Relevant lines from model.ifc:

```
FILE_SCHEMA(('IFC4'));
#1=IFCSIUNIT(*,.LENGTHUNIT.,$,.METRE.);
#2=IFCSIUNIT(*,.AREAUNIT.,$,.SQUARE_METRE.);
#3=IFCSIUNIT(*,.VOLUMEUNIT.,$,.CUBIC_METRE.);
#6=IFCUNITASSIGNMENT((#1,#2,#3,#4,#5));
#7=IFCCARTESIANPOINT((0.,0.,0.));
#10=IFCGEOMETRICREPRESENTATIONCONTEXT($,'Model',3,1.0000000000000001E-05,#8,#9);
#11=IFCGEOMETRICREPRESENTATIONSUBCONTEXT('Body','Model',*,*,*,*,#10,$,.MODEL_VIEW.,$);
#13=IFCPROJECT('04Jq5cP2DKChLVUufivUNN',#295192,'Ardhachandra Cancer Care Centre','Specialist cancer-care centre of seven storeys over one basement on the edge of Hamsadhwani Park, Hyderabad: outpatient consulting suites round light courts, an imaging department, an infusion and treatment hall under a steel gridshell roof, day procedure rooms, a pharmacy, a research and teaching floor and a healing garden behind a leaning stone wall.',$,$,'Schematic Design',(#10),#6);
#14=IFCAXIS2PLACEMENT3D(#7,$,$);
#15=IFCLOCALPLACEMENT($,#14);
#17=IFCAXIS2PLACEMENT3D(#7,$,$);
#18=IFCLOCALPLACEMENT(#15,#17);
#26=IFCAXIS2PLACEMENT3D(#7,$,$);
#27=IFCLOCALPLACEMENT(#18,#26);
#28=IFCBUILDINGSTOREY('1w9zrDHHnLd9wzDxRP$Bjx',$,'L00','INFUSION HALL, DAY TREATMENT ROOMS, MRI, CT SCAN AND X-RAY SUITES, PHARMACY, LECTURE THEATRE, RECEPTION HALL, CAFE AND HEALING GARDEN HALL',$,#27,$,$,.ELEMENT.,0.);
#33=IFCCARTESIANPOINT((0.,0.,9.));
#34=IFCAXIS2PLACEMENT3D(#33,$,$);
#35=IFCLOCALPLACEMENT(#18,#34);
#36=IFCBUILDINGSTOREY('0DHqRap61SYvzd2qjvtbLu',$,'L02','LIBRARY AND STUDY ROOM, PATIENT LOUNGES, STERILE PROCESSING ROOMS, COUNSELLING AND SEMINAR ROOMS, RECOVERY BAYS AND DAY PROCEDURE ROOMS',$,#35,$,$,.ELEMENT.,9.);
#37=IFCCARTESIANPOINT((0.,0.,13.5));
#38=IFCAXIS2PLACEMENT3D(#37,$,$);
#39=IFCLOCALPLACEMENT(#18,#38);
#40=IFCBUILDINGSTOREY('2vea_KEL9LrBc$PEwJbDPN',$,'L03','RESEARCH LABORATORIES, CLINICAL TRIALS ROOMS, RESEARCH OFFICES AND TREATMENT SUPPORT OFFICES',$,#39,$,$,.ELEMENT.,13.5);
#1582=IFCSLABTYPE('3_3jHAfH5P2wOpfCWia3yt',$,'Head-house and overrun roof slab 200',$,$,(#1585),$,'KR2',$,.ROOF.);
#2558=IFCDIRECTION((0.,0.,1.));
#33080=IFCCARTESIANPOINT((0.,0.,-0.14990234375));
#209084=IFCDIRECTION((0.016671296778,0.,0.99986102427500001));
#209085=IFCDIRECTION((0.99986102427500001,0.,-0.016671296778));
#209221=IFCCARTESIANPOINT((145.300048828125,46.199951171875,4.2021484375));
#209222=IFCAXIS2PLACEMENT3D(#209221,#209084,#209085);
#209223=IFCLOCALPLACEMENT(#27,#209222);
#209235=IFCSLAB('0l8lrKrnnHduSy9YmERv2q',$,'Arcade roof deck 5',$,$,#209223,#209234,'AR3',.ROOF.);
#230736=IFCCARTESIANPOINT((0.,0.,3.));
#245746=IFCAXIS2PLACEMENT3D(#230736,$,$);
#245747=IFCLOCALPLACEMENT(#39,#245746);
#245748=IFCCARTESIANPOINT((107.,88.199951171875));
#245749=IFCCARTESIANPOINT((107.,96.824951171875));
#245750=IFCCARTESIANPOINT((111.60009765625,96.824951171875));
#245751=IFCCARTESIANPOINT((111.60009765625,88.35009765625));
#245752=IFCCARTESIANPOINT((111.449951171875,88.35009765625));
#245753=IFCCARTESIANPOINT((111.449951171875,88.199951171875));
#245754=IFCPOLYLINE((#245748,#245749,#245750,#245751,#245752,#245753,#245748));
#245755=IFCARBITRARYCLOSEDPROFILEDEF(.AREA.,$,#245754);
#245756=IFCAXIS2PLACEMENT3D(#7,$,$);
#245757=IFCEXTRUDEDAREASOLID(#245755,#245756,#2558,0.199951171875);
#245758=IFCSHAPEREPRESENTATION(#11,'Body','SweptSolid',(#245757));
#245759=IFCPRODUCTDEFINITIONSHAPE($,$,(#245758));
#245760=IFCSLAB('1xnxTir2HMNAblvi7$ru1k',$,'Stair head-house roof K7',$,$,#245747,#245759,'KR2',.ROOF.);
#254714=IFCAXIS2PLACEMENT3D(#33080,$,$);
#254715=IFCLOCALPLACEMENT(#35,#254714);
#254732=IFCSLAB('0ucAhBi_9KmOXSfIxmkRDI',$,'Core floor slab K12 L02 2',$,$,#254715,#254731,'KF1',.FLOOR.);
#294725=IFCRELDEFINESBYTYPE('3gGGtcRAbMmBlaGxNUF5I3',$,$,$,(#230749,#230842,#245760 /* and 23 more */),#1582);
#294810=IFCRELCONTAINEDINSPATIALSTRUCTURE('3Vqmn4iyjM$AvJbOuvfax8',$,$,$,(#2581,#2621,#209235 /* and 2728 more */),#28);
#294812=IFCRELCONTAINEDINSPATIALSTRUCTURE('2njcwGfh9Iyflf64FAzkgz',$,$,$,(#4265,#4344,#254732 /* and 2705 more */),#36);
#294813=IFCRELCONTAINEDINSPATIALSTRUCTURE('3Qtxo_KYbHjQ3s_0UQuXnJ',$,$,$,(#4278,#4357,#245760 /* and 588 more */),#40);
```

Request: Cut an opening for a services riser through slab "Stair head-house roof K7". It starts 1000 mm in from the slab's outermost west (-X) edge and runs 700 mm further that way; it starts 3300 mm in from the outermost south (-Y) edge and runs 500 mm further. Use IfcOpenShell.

```python
import numpy as np
import ifcopenshell
import ifcopenshell.api.feature
import ifcopenshell.api.geometry
import ifcopenshell.api.root
import ifcopenshell.geom
import ifcopenshell.util.placement
import ifcopenshell.util.representation
import ifcopenshell.util.shape
import ifcopenshell.util.unit

model = ifcopenshell.open("model.ifc")
unit_scale = ifcopenshell.util.unit.calculate_unit_scale(model)
settings = ifcopenshell.geom.settings()


def volume(element):
    """Net volume in cubic metres, openings subtracted."""
    shape = ifcopenshell.geom.create_shape(settings, element)
    return ifcopenshell.util.shape.get_volume(shape.geometry)


slab = model.by_guid("1xnxTir2HMNAblvi7$ru1k")
before = volume(slab)

# Extent in the slab's own axes, in metres. The edges named are its -X and -Y sides.
slab_shape = ifcopenshell.geom.create_shape(settings, slab)
vertices = ifcopenshell.util.shape.get_vertices(slab_shape.geometry)
x_min, y_min, bottom = vertices.min(axis=0)
top = vertices[:, 2].max()

opening = ifcopenshell.api.root.create_entity(model, ifc_class="IfcOpeningElement", name="Services riser opening", predefined_type="OPENING")
context = ifcopenshell.util.representation.get_context(model, "Model", "Body", "MODEL_VIEW")
width, depth = 0.7, 0.5
outline = [(0.0, 0.0), (width, 0.0), (width, depth), (0.0, depth), (0.0, 0.0)]
# Overshoot both faces by 50 mm so the cut is clean.
shape = ifcopenshell.api.geometry.add_slab_representation(
    model, context=context, depth=top - bottom + 0.1, polyline=outline
)
ifcopenshell.api.geometry.assign_representation(model, product=opening, representation=shape)

matrix = ifcopenshell.util.placement.get_local_placement(slab.ObjectPlacement)
matrix[:, 3] = matrix @ np.append(np.array([x_min + 1, y_min + 3.3, bottom - 0.05]) / unit_scale, 1.0)
ifcopenshell.api.geometry.edit_object_placement(model, product=opening, matrix=matrix, is_si=False)
ifcopenshell.api.feature.add_feature(model, feature=opening, element=slab)

after = volume(slab)

print(f"slab volume {before:.3f} -> {after:.3f} m3")

model.write("model_rev.ifc")
```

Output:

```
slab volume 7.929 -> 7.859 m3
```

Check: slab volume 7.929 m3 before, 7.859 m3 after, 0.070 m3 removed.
